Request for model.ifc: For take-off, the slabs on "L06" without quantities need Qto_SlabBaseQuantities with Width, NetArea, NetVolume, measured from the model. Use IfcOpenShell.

First a look at what the model holds.

```python
import ifcopenshell
import ifcopenshell.util.element
import ifcopenshell.util.unit

model = ifcopenshell.open("model.ifc")
print(model.schema)
for unit_type in ("LENGTHUNIT", "AREAUNIT", "VOLUMEUNIT"):
    print(unit_type, ifcopenshell.util.unit.calculate_unit_scale(model, unit_type))
storey = next(s for s in model.by_type("IfcBuildingStorey") if s.Name == "L06")
slabs = [e for e in ifcopenshell.util.element.get_decomposition(storey) if e.is_a("IfcSlab")]
for e in sorted(slabs, key=lambda e: e.id()):
    print(e.id(), e.is_a(), e.Name, list(ifcopenshell.util.element.get_psets(e, qtos_only=True)), sep=" | ")
```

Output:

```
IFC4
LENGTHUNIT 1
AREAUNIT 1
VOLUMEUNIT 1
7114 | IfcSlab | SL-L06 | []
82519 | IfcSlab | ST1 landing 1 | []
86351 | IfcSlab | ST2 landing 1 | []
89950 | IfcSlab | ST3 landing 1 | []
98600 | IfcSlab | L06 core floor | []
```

```python
import ifcopenshell
import ifcopenshell.api.pset
import ifcopenshell.geom
import ifcopenshell.util.element
import ifcopenshell.util.shape
import ifcopenshell.util.unit

model = ifcopenshell.open("model.ifc")
unit_scale = ifcopenshell.util.unit.calculate_unit_scale(model)
area_scale = ifcopenshell.util.unit.calculate_unit_scale(model, "AREAUNIT")
volume_scale = ifcopenshell.util.unit.calculate_unit_scale(model, "VOLUMEUNIT")
settings = ifcopenshell.geom.settings()

storey = next(s for s in model.by_type("IfcBuildingStorey") if s.Name == "L06")
slabs = [e for e in ifcopenshell.util.element.get_decomposition(storey) if e.is_a("IfcSlab")]

for e in sorted(slabs, key=lambda e: e.id()):
    if ifcopenshell.util.element.get_psets(e, qtos_only=True, should_inherit=False):
        continue
    # Geometry comes back in metres, in the element's own axes.
    shape = ifcopenshell.geom.create_shape(settings, e)
    values = {
        "Width": ifcopenshell.util.shape.get_z(shape.geometry) / unit_scale,
        "NetArea": ifcopenshell.util.shape.get_footprint_area(shape.geometry) / area_scale,
        "NetVolume": ifcopenshell.util.shape.get_volume(shape.geometry) / volume_scale,
    }
    qto = ifcopenshell.api.pset.add_qto(model, product=e, name="Qto_SlabBaseQuantities")
    ifcopenshell.api.pset.edit_qto(model, qto=qto, properties=values)
    print(e.id(), {k: round(v, 3) for k, v in values.items()})

model.write("model-out.ifc")
```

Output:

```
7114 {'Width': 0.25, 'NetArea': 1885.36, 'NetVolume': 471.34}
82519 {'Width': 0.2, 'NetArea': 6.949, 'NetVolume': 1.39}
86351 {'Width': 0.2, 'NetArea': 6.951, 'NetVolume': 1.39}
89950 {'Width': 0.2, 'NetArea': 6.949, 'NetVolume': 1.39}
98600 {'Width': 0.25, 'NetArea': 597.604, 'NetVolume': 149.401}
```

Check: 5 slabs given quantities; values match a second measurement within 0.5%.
